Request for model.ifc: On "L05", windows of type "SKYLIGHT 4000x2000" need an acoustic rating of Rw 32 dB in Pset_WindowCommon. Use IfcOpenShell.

First a look at what the model holds.

```python
import ifcopenshell
import ifcopenshell.util.element

model = ifcopenshell.open("model.ifc")
print(model.schema)
storey = next(s for s in model.by_type("IfcBuildingStorey") if s.Name == "L05")
windows = [e for e in ifcopenshell.util.element.get_decomposition(storey) if e.is_a("IfcWindow")]
seen = {}
for e in windows:
    element_type = ifcopenshell.util.element.get_type(e)
    key = (element_type.Name if element_type != e and element_type else None, ifcopenshell.util.element.get_pset(e, "Pset_WindowCommon", "AcousticRating"))
    seen[key] = seen.get(key, 0) + 1
for (name, value), count in sorted(seen.items(), key=str):
    print(count, "x", name, "|", value)
```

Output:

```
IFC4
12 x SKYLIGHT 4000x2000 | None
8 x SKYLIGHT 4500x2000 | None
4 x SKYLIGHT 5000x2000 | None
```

```python
import ifcopenshell
import ifcopenshell.api.pset
import ifcopenshell.util.element

model = ifcopenshell.open("model.ifc")

storey = next(s for s in model.by_type("IfcBuildingStorey") if s.Name == "L05")
windows = [e for e in ifcopenshell.util.element.get_decomposition(storey) if e.is_a("IfcWindow")]

count = 0
for e in windows:
    element_type = ifcopenshell.util.element.get_type(e)
    if element_type in (None, e) or element_type.Name != "SKYLIGHT 4000x2000":
        continue
    # add_pset returns the element's existing set when there is one.
    pset = ifcopenshell.api.pset.add_pset(model, product=e, name="Pset_WindowCommon")
    ifcopenshell.api.pset.edit_pset(model, pset=pset, properties={"AcousticRating": "Rw 32 dB"})
    count += 1

print(count, "windows updated")

model.write("model-out.ifc")
```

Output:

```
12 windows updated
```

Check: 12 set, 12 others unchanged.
